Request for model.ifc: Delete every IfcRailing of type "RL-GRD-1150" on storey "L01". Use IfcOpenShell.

First a look at what the model holds.

```python
import ifcopenshell
import ifcopenshell.util.element

model = ifcopenshell.open("model.ifc")
print(model.schema)
storey = next(s for s in model.by_type("IfcBuildingStorey") if s.Name == "L01")
railings = [e for e in ifcopenshell.util.element.get_decomposition(storey) if e.is_a("IfcRailing")]
seen = {}
for e in railings:
    element_type = ifcopenshell.util.element.get_type(e)
    name = element_type.Name if element_type not in (None, e) else None
    seen[name] = seen.get(name, 0) + 1
for name, count in sorted(seen.items(), key=str):
    print(count, "x", name)
```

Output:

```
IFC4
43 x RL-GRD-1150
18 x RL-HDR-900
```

```python
import ifcopenshell
import ifcopenshell.api.root
import ifcopenshell.util.element

model = ifcopenshell.open("model.ifc")

storey = next(s for s in model.by_type("IfcBuildingStorey") if s.Name == "L01")
railings = [e for e in ifcopenshell.util.element.get_decomposition(storey) if e.is_a("IfcRailing")]
targets = [e for e in railings if (t := ifcopenshell.util.element.get_type(e)) not in (None, e) and t.Name == "RL-GRD-1150"]

for e in targets:
    ifcopenshell.api.root.remove_product(model, product=e)
print(len(targets), "removed")

model.write("model_v2.ifc")
```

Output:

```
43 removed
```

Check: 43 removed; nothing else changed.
